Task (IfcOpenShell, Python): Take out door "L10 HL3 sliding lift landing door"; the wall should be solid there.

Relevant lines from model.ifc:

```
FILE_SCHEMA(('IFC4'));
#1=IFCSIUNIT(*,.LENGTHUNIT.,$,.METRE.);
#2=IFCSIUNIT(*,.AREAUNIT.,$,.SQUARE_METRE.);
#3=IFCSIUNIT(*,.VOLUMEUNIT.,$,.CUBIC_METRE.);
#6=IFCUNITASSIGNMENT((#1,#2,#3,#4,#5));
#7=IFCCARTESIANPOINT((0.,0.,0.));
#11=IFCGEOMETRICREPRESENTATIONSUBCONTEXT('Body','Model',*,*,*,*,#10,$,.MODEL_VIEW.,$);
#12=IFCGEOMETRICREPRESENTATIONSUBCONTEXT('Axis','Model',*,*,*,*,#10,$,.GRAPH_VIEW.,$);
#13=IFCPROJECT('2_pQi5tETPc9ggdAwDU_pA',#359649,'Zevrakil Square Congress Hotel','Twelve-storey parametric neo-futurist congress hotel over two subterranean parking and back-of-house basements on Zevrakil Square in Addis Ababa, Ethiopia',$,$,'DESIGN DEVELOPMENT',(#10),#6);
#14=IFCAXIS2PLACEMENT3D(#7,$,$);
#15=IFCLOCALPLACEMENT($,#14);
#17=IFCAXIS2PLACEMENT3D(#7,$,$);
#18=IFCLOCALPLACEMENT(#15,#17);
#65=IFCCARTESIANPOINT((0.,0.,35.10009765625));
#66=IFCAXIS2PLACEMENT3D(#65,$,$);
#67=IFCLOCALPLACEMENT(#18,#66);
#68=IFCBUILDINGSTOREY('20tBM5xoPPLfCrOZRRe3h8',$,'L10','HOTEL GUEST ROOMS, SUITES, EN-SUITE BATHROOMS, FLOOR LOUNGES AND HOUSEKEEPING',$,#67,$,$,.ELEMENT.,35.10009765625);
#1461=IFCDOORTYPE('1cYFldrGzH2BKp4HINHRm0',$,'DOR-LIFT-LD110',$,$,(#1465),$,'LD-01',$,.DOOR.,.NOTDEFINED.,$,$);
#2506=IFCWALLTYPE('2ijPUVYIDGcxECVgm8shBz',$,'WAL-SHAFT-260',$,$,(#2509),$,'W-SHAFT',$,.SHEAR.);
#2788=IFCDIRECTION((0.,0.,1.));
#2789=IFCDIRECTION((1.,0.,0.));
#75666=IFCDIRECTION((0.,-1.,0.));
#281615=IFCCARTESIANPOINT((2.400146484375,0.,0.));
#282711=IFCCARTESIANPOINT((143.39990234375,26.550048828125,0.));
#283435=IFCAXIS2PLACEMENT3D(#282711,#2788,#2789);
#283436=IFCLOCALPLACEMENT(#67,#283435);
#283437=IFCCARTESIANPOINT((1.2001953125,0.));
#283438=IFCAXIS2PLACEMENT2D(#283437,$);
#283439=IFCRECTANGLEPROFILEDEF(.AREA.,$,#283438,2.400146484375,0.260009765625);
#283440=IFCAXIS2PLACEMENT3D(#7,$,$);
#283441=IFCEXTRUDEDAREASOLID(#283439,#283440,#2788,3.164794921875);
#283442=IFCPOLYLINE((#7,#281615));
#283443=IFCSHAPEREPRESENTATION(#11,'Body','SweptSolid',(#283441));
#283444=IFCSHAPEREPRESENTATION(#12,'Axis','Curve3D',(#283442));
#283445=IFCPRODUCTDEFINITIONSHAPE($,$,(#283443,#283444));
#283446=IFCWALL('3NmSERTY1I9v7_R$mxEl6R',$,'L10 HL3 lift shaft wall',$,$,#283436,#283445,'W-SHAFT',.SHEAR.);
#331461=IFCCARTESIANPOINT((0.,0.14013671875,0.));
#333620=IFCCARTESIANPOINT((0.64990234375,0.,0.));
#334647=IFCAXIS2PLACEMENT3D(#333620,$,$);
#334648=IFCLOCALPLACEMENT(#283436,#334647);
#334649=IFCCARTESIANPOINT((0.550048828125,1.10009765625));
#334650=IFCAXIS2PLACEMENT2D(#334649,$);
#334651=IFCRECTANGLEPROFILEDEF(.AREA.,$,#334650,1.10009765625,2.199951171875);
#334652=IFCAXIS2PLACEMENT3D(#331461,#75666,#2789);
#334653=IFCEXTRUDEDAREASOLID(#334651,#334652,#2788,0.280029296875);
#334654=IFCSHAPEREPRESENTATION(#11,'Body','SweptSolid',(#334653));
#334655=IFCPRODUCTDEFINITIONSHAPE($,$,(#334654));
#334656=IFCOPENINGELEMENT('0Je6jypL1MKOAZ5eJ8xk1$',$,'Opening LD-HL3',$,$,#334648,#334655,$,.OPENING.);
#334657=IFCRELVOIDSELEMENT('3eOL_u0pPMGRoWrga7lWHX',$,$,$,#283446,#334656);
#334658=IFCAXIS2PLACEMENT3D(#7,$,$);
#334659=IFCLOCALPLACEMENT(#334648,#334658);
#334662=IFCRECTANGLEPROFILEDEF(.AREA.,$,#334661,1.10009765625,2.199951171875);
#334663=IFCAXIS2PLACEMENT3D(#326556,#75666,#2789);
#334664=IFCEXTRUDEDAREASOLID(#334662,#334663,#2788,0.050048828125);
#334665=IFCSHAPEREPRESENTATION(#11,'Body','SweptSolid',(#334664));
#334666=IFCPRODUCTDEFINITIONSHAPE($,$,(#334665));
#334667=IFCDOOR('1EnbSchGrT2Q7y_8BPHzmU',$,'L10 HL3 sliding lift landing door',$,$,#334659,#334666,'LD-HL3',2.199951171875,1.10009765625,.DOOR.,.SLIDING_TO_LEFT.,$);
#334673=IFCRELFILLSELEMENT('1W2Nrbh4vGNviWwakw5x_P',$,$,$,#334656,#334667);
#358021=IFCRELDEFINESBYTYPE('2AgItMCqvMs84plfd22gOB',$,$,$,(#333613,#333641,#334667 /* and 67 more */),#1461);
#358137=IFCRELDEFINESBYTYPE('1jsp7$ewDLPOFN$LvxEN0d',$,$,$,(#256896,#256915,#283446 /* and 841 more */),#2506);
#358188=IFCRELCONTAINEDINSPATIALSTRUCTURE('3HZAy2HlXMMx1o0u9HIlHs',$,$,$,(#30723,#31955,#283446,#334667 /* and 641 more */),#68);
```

```python
import ifcopenshell
import ifcopenshell.api.feature
import ifcopenshell.api.root
import ifcopenshell.geom
import ifcopenshell.util.shape

model = ifcopenshell.open("model.ifc")
settings = ifcopenshell.geom.settings()


def volume(element):
    """Net volume in cubic metres, openings subtracted."""
    shape = ifcopenshell.geom.create_shape(settings, element)
    return ifcopenshell.util.shape.get_volume(shape.geometry)


door = model.by_guid("1EnbSchGrT2Q7y_8BPHzmU")
opening = door.FillsVoids[0].RelatingOpeningElement
wall = opening.VoidsElements[0].RelatingBuildingElement
before = volume(wall)

ifcopenshell.api.root.remove_product(model, product=door)
ifcopenshell.api.feature.remove_feature(model, feature=opening)

after = volume(wall)

print(f"wall volume {before:.3f} -> {after:.3f} m3")

model.write("model_edited.ifc")
```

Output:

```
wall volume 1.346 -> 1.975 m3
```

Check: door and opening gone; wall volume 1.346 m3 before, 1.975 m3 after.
